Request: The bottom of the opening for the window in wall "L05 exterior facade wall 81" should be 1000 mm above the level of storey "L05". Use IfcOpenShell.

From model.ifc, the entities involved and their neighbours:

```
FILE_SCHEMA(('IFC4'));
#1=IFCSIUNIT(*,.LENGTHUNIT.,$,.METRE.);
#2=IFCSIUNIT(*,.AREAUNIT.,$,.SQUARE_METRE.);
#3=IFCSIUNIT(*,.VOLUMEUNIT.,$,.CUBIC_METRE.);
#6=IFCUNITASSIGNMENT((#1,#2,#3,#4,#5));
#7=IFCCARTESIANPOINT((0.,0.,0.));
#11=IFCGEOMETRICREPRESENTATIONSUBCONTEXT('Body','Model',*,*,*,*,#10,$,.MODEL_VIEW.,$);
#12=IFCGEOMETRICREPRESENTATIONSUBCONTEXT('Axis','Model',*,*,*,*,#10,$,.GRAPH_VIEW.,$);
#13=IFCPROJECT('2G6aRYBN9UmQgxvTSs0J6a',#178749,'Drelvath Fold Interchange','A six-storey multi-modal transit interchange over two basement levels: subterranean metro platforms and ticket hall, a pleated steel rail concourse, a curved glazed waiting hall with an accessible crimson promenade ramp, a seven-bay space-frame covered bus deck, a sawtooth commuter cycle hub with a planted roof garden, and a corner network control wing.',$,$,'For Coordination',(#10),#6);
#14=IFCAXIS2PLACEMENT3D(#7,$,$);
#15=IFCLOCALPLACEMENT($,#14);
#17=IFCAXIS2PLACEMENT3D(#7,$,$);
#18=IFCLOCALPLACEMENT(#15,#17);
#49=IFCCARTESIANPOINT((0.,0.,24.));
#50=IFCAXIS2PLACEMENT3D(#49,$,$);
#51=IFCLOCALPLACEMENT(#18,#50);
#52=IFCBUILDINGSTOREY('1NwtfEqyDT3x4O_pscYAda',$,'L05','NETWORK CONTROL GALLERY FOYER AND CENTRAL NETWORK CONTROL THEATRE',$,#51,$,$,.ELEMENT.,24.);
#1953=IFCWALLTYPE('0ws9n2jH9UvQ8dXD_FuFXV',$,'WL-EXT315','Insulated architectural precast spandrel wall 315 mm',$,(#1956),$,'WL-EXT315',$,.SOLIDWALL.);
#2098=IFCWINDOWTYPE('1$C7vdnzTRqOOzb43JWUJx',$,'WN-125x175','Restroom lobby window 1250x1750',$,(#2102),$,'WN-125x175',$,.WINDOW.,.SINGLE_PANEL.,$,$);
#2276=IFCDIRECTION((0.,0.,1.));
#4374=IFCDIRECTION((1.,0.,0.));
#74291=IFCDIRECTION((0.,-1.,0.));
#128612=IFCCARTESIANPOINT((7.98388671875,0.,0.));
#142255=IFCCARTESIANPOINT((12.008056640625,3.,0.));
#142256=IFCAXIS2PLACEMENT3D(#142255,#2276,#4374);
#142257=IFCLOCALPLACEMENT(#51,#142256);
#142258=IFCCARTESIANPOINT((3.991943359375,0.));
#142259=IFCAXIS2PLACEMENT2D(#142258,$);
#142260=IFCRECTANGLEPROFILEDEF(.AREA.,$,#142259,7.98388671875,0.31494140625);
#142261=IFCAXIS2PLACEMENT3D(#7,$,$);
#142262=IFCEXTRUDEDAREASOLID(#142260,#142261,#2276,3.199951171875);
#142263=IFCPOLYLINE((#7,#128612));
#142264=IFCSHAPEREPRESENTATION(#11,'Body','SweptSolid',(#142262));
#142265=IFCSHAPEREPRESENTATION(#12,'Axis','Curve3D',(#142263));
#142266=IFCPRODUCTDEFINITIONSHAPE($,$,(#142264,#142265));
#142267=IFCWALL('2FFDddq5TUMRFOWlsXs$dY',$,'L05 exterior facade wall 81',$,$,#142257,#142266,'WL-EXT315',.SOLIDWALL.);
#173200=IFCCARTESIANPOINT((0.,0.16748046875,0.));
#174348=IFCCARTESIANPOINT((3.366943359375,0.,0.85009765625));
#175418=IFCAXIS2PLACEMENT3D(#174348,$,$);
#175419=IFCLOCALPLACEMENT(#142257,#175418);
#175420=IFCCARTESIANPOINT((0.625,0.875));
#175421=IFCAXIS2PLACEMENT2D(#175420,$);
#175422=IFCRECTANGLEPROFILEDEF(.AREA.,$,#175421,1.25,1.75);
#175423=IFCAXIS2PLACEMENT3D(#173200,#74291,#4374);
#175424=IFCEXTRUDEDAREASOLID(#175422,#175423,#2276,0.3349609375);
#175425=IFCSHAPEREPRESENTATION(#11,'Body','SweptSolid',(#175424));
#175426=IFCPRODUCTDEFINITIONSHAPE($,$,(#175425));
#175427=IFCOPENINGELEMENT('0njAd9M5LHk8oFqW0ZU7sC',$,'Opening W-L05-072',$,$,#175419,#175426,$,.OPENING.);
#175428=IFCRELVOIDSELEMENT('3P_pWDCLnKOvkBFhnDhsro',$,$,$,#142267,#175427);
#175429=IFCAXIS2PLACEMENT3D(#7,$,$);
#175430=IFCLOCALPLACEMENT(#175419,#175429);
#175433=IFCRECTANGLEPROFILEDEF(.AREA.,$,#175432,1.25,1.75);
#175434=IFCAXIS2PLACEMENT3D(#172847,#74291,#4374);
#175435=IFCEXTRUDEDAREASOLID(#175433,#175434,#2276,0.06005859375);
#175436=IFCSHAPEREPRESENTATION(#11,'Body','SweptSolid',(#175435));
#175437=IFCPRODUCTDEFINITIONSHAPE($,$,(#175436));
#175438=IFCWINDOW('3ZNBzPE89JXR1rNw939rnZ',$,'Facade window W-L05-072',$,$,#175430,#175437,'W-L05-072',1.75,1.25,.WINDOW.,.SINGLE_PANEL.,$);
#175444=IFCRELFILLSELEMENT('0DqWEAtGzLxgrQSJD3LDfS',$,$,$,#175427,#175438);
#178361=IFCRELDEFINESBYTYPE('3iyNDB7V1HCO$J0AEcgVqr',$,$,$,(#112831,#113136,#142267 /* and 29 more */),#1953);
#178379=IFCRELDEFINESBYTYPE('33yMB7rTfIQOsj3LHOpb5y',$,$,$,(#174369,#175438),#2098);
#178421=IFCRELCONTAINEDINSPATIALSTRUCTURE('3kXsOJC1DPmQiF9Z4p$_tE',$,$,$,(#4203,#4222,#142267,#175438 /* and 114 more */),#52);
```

```python
import numpy as np
import ifcopenshell
import ifcopenshell.api.geometry
import ifcopenshell.geom
import ifcopenshell.util.element
import ifcopenshell.util.placement
import ifcopenshell.util.shape
import ifcopenshell.util.unit

model = ifcopenshell.open("model.ifc")
unit_scale = ifcopenshell.util.unit.calculate_unit_scale(model)

window = model.by_guid("3ZNBzPE89JXR1rNw939rnZ")
opening = window.FillsVoids[0].RelatingOpeningElement
storey = ifcopenshell.util.element.get_container(window, ifc_class="IfcBuildingStorey")
level = ifcopenshell.util.placement.get_local_placement(storey.ObjectPlacement)[2, 3]

# The opening's origin need not be at the sill, so measure its lowest point.
shape = ifcopenshell.geom.create_shape(ifcopenshell.geom.settings(), opening)
bottom = ifcopenshell.util.shape.get_shape_bottom_elevation(shape, shape.geometry) / unit_scale
dz = level + 1.0 - bottom

shift = np.array([0.0, 0.0, dz])
# The window is placed relative to its opening, so it follows when the opening moves.
matrix = ifcopenshell.util.placement.get_local_placement(opening.ObjectPlacement)
matrix[:3, 3] += shift
ifcopenshell.api.geometry.edit_object_placement(
    model, product=opening, matrix=matrix, is_si=False, should_transform_children=True
)

print(f"moved by {dz * unit_scale:+.3f} m")

model.write("model_rev.ifc")
```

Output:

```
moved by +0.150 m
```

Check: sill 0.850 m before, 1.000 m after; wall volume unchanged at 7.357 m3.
